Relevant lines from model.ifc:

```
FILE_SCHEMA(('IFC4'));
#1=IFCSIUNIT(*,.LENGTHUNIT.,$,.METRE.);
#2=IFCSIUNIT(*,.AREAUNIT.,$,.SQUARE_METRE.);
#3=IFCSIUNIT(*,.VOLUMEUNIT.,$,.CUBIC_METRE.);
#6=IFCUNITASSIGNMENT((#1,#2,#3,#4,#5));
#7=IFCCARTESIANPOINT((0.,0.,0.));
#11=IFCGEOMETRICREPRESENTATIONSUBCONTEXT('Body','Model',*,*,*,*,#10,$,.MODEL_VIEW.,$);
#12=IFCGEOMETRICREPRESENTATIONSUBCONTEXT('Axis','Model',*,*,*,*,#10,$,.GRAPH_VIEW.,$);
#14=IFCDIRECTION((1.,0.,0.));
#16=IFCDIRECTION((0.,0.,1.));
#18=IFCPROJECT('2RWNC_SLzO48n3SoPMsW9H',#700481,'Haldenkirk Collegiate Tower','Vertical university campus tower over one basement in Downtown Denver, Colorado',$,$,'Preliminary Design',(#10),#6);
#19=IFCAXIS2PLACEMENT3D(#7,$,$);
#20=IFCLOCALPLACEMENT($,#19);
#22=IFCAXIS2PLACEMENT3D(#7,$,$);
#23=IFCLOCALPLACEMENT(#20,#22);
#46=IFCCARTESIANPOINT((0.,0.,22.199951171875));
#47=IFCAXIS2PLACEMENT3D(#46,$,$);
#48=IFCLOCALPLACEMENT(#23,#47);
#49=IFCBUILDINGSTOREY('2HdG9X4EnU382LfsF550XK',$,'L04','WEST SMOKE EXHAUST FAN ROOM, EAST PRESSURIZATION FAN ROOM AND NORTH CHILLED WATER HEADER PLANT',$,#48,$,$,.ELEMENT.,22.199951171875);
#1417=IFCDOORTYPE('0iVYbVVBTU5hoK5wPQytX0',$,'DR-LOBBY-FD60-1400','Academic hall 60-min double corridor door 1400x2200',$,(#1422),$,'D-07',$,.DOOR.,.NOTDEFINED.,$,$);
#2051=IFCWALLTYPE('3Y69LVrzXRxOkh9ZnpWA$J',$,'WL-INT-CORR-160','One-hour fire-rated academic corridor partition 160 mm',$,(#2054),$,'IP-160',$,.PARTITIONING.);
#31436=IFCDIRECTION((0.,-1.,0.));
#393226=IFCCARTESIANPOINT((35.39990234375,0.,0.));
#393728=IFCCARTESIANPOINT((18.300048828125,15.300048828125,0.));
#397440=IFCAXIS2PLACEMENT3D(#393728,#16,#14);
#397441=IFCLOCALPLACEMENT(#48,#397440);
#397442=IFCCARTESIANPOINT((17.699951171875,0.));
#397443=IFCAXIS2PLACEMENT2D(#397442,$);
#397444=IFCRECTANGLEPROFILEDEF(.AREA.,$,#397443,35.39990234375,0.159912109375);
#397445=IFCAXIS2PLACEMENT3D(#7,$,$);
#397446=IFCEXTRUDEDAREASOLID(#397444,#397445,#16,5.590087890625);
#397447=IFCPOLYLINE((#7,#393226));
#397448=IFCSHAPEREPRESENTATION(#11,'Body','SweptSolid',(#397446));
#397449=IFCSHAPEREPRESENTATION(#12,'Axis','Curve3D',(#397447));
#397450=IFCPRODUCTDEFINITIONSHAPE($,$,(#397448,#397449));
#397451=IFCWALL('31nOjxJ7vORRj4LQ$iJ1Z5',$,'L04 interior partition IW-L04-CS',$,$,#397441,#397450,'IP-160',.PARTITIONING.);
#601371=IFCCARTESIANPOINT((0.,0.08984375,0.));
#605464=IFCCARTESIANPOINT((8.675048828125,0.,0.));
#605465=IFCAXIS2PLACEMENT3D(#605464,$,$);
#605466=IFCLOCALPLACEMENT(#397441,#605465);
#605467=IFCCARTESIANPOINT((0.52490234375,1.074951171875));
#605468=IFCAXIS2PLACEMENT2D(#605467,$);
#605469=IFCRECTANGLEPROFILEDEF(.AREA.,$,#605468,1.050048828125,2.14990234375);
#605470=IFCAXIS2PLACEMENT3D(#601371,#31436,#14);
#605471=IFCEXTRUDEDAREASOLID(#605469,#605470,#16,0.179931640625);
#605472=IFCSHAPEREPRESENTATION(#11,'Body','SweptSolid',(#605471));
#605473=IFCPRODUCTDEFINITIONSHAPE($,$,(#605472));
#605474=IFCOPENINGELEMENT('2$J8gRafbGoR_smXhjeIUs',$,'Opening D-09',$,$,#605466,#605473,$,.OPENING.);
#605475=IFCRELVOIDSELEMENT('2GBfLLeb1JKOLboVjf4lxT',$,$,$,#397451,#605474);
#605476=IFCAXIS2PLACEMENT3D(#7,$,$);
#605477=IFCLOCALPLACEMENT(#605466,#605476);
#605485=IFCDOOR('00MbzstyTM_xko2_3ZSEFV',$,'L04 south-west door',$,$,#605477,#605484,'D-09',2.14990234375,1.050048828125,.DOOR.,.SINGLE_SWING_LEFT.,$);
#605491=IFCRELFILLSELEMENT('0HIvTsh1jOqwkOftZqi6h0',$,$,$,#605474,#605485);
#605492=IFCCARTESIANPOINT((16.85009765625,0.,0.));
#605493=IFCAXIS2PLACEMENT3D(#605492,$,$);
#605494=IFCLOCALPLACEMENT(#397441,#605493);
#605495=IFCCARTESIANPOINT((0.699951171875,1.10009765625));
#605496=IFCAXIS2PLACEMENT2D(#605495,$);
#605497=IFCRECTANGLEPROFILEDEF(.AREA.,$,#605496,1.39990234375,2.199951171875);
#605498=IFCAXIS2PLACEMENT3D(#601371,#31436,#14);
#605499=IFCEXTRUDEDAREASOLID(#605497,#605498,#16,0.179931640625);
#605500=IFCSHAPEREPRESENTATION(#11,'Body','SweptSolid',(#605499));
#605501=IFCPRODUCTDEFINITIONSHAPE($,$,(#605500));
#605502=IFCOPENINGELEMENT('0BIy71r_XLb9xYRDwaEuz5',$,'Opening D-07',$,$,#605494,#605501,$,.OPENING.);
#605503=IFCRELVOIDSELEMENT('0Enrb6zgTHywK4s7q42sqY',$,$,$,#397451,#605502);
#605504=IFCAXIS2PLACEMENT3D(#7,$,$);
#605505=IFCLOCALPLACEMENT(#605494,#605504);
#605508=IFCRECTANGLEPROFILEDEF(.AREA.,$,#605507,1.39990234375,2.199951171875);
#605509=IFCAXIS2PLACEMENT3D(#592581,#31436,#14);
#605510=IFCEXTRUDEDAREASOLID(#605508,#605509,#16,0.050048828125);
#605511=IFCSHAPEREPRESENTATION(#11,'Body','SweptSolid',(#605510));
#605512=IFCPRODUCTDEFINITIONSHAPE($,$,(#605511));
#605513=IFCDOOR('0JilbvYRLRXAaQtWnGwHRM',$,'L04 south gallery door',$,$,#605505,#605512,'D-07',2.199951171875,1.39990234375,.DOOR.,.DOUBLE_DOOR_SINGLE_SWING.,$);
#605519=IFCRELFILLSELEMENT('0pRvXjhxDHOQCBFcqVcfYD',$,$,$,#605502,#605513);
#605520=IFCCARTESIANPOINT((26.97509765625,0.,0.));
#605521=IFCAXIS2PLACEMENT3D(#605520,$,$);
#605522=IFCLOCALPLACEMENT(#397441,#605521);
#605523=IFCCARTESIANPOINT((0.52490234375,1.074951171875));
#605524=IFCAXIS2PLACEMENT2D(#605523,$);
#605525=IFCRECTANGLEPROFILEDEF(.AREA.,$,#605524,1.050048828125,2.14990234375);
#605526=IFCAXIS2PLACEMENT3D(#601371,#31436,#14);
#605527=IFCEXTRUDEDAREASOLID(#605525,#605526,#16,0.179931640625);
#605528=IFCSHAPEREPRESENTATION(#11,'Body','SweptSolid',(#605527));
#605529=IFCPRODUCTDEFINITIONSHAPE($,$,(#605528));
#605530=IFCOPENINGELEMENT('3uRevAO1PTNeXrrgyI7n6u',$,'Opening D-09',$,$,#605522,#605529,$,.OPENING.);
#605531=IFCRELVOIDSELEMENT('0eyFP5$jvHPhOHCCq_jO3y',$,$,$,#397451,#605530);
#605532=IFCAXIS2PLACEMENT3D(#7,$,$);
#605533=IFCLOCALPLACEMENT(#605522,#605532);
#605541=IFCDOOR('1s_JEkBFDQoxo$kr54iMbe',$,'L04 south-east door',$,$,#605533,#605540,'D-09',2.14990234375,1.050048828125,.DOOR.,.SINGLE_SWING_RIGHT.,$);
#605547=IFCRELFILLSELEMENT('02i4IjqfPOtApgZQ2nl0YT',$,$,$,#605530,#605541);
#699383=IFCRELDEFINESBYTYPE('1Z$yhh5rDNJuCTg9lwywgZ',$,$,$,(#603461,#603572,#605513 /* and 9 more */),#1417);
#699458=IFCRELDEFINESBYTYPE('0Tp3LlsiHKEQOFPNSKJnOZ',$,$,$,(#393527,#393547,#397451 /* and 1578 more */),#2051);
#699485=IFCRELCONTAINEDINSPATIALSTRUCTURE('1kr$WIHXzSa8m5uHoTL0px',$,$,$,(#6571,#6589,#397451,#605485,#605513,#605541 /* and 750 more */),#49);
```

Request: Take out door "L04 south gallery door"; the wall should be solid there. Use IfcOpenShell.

```python
import ifcopenshell
import ifcopenshell.api.feature
import ifcopenshell.api.root
import ifcopenshell.geom
import ifcopenshell.util.shape

model = ifcopenshell.open("model.ifc")
settings = ifcopenshell.geom.settings()


def volume(element):
    """Net volume in cubic metres, openings subtracted."""
    shape = ifcopenshell.geom.create_shape(settings, element)
    return ifcopenshell.util.shape.get_volume(shape.geometry)


door = model.by_guid("0JilbvYRLRXAaQtWnGwHRM")
opening = door.FillsVoids[0].RelatingOpeningElement
wall = opening.VoidsElements[0].RelatingBuildingElement
before = volume(wall)

ifcopenshell.api.root.remove_product(model, product=door)
ifcopenshell.api.feature.remove_feature(model, feature=opening)

after = volume(wall)

print(f"wall volume {before:.3f} -> {after:.3f} m3")

model.write("model_edited.ifc")
```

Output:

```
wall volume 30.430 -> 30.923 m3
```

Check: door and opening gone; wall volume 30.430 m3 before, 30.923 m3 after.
